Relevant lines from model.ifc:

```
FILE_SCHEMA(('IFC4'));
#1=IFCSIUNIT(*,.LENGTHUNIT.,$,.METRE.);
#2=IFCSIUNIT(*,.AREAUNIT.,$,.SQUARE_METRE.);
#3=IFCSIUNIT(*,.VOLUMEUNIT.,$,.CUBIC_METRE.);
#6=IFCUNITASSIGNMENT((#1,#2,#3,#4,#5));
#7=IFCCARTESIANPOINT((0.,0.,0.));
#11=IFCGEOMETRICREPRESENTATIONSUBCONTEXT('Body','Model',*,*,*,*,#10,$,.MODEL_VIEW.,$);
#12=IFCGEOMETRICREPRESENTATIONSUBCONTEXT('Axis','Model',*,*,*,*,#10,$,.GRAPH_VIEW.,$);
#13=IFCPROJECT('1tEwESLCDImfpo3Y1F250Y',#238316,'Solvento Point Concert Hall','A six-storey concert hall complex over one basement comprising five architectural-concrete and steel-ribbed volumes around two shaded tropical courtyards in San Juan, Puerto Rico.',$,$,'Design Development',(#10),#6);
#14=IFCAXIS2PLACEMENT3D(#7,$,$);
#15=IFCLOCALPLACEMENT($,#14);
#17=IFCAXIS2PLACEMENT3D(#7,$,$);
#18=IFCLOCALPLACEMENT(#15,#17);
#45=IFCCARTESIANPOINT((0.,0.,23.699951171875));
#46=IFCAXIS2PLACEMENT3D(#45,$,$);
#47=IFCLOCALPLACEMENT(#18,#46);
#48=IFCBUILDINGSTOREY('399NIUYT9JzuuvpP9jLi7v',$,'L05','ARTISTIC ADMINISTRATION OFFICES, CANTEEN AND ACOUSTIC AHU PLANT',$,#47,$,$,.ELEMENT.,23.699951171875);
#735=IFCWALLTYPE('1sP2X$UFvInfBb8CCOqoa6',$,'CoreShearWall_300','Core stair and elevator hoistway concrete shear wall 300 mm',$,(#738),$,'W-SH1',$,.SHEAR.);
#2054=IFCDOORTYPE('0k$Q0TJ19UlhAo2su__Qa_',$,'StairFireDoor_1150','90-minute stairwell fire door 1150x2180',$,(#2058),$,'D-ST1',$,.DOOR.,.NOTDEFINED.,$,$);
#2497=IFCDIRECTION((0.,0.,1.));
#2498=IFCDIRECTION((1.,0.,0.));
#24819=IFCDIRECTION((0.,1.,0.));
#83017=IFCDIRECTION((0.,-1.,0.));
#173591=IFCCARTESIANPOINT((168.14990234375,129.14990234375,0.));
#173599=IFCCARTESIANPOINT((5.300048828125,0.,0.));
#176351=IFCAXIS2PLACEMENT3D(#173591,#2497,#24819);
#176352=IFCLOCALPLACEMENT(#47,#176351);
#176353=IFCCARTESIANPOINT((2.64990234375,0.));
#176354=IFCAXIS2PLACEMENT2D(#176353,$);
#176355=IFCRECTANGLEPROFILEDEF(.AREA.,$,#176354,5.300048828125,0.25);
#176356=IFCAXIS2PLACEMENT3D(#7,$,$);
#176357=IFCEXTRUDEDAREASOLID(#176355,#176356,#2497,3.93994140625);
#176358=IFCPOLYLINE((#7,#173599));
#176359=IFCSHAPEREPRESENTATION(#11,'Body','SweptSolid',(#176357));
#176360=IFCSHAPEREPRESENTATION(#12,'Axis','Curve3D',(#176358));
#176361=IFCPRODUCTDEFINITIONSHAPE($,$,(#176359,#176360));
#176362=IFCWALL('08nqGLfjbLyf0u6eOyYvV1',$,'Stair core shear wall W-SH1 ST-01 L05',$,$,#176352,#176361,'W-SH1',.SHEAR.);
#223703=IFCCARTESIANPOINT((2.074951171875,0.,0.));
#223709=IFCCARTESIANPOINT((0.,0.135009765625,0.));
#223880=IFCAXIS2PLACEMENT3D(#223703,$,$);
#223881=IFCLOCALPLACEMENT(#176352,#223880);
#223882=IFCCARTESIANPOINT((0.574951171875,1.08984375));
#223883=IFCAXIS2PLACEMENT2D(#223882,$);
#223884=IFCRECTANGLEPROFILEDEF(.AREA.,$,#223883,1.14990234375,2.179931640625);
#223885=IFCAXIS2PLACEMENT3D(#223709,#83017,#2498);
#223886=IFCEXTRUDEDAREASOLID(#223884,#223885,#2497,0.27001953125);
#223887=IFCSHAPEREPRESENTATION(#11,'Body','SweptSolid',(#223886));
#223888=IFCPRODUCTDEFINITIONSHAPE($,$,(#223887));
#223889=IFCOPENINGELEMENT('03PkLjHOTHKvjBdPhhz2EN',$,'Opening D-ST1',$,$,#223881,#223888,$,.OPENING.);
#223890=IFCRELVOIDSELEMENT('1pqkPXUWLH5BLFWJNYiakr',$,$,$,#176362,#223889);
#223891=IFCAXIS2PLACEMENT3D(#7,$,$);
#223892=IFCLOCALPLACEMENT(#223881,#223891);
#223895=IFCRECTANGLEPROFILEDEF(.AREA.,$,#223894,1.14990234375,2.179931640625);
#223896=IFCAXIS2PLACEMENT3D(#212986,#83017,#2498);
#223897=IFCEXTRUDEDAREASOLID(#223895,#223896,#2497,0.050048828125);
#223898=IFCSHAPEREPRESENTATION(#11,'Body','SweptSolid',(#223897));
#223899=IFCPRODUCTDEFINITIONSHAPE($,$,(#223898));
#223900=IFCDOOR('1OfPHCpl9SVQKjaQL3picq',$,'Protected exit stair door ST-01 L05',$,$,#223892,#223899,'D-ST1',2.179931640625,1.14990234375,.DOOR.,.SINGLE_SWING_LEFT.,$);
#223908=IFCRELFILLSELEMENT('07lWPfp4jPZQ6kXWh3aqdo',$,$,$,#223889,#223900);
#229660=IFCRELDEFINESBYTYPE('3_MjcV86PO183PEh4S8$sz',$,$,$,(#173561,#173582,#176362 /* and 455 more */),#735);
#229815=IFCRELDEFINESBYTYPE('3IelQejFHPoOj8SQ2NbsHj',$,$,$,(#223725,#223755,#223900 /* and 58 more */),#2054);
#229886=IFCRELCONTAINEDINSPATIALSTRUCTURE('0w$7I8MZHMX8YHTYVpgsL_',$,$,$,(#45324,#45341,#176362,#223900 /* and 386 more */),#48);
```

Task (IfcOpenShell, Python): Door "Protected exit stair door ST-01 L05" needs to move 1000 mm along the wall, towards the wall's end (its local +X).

```python
import ifcopenshell
import ifcopenshell.api.geometry
import ifcopenshell.util.placement

model = ifcopenshell.open("model.ifc")

door = model.by_guid("1OfPHCpl9SVQKjaQL3picq")
opening = door.FillsVoids[0].RelatingOpeningElement
wall = opening.VoidsElements[0].RelatingBuildingElement

wall_matrix = ifcopenshell.util.placement.get_local_placement(wall.ObjectPlacement)
shift = wall_matrix[:3, 0] * 1.0
before = ifcopenshell.util.placement.get_local_placement(door.ObjectPlacement)[:3, 3].copy()

# The door is placed relative to its opening, so it follows when the opening moves.
matrix = ifcopenshell.util.placement.get_local_placement(opening.ObjectPlacement)
matrix[:3, 3] += shift
ifcopenshell.api.geometry.edit_object_placement(
    model, product=opening, matrix=matrix, is_si=False, should_transform_children=True
)

after = ifcopenshell.util.placement.get_local_placement(door.ObjectPlacement)[:3, 3]
print("door moved by", (after - before).round(3) + 0.0)

model.write("model_rev.ifc")
```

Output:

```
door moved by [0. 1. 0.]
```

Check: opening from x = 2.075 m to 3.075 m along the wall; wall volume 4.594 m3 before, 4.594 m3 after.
